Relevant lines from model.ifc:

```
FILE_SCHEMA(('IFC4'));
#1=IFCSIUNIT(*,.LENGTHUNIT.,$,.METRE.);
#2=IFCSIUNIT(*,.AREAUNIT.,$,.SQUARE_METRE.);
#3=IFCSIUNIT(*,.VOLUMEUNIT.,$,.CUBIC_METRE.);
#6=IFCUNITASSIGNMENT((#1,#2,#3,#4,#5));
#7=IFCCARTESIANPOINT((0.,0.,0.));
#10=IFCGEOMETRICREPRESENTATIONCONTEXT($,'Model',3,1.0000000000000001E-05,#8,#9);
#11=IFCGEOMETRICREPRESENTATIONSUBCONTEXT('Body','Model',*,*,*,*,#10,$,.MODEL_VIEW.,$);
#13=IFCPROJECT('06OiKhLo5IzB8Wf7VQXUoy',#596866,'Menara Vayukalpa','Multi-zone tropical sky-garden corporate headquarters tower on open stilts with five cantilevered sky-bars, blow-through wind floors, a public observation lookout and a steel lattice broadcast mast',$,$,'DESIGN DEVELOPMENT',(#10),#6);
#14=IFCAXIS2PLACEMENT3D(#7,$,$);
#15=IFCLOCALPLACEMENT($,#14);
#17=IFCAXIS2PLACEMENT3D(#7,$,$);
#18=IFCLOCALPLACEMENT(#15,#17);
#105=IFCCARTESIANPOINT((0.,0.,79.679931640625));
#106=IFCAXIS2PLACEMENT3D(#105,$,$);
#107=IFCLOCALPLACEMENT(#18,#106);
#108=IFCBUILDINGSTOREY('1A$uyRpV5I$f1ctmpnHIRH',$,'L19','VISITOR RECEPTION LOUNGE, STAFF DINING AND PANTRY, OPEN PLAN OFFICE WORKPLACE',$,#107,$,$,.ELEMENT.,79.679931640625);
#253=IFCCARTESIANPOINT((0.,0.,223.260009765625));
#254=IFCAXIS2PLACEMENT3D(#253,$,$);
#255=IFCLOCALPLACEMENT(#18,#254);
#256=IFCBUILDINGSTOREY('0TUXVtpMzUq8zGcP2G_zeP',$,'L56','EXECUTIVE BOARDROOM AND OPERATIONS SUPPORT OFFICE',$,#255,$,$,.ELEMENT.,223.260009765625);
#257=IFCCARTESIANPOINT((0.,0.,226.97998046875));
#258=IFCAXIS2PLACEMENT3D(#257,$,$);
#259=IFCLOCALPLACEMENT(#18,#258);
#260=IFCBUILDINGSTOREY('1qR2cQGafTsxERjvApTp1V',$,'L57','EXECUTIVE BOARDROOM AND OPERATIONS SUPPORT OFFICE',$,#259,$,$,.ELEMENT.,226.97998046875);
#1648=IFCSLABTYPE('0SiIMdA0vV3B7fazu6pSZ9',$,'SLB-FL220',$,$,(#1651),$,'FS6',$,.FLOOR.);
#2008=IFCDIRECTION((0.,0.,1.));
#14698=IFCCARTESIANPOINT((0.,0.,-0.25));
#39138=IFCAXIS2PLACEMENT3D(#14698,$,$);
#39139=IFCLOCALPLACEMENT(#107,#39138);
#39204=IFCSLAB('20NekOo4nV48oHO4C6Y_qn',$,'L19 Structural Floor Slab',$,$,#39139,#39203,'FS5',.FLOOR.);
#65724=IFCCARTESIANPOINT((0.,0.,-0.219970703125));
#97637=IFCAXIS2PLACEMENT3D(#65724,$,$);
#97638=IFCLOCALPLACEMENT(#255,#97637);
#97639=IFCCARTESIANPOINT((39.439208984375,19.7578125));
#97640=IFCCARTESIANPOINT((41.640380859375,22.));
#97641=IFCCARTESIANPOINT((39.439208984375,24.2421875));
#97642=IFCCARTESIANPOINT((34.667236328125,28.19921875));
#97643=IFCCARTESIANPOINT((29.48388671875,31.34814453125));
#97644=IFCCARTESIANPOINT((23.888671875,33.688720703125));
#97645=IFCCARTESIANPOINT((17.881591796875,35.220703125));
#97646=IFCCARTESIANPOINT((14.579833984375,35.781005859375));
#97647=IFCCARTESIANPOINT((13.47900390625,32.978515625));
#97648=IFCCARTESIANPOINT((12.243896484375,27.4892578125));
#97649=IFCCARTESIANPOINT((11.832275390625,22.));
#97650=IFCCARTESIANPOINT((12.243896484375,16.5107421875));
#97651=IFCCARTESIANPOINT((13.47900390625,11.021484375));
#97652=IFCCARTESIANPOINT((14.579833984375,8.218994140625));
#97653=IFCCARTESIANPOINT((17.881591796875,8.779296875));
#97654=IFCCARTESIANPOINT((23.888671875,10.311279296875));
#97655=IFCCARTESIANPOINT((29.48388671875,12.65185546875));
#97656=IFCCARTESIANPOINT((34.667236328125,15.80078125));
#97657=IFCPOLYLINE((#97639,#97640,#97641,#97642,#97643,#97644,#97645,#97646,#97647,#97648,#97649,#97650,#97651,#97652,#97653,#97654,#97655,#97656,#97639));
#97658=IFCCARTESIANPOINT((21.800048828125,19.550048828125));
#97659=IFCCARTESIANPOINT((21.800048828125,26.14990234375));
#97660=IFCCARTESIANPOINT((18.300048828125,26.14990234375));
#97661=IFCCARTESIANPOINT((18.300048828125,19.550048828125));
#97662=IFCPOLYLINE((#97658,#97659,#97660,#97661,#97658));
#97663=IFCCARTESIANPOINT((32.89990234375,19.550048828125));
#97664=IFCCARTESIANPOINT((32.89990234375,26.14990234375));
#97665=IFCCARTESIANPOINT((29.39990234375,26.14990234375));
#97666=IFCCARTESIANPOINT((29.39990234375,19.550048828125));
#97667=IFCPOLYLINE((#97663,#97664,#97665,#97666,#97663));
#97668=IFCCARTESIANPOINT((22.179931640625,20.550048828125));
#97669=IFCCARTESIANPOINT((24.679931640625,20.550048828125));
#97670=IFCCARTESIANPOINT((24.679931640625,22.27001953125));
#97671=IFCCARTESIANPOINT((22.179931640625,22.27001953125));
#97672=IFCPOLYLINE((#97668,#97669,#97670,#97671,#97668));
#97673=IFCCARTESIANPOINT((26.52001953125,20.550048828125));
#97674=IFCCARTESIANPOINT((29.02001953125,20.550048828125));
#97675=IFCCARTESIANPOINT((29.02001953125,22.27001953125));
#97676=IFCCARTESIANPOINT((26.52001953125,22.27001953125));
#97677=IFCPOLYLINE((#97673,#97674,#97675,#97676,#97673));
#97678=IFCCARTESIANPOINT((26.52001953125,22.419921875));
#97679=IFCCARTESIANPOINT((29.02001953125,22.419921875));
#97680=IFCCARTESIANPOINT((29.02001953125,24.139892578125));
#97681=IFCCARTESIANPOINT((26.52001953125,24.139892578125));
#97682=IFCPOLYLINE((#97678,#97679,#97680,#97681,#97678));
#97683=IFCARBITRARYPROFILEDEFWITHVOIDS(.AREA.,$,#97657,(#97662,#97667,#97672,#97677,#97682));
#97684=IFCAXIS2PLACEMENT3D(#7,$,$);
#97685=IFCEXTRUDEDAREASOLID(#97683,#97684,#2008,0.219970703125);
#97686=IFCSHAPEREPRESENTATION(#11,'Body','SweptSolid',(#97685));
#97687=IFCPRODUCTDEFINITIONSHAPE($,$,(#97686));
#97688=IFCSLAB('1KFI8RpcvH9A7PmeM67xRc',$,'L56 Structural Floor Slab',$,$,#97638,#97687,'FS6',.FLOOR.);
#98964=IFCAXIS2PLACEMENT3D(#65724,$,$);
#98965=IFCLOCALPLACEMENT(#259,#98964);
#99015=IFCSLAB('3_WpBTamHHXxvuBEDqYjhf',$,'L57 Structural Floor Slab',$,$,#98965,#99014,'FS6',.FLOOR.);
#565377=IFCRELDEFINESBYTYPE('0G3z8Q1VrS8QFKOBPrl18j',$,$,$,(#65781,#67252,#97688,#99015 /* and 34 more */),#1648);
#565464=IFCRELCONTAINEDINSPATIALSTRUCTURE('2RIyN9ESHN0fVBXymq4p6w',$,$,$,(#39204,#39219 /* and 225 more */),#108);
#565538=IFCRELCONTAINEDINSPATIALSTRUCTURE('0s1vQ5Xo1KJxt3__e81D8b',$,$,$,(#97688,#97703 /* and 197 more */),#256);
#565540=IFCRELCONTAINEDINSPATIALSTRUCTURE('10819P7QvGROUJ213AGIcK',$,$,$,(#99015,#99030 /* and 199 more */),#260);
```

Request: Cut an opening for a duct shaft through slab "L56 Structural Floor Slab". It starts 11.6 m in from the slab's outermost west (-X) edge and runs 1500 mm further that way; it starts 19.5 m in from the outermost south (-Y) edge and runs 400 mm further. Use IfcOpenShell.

```python
import numpy as np
import ifcopenshell
import ifcopenshell.api.feature
import ifcopenshell.api.geometry
import ifcopenshell.api.root
import ifcopenshell.geom
import ifcopenshell.util.placement
import ifcopenshell.util.representation
import ifcopenshell.util.shape
import ifcopenshell.util.unit

model = ifcopenshell.open("model.ifc")
unit_scale = ifcopenshell.util.unit.calculate_unit_scale(model)
settings = ifcopenshell.geom.settings()


def volume(element):
    """Net volume in cubic metres, openings subtracted."""
    shape = ifcopenshell.geom.create_shape(settings, element)
    return ifcopenshell.util.shape.get_volume(shape.geometry)


slab = model.by_id(97688)
before = volume(slab)

# Extent in the slab's own axes, in metres. The edges named are its -X and -Y sides.
slab_shape = ifcopenshell.geom.create_shape(settings, slab)
vertices = ifcopenshell.util.shape.get_vertices(slab_shape.geometry)
x_min, y_min, bottom = vertices.min(axis=0)
top = vertices[:, 2].max()

opening = ifcopenshell.api.root.create_entity(model, ifc_class="IfcOpeningElement", name="Duct shaft opening", predefined_type="OPENING")
context = ifcopenshell.util.representation.get_context(model, "Model", "Body", "MODEL_VIEW")
width, depth = 1.5, 0.4
outline = [(0.0, 0.0), (width, 0.0), (width, depth), (0.0, depth), (0.0, 0.0)]
# Overshoot both faces by 50 mm so the cut is clean.
shape = ifcopenshell.api.geometry.add_slab_representation(
    model, context=context, depth=top - bottom + 0.1, polyline=outline
)
ifcopenshell.api.geometry.assign_representation(model, product=opening, representation=shape)

matrix = ifcopenshell.util.placement.get_local_placement(slab.ObjectPlacement)
matrix[:, 3] = matrix @ np.append(np.array([x_min + 11.6, y_min + 19.5, bottom - 0.05]) / unit_scale, 1.0)
ifcopenshell.api.geometry.edit_object_placement(model, product=opening, matrix=matrix, is_si=False)
ifcopenshell.api.feature.add_feature(model, feature=opening, element=slab)

after = volume(slab)

print(f"slab volume {before:.3f} -> {after:.3f} m3")

model.write("model_v2.ifc")
```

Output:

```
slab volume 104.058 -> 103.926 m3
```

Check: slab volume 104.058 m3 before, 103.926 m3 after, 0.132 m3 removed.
